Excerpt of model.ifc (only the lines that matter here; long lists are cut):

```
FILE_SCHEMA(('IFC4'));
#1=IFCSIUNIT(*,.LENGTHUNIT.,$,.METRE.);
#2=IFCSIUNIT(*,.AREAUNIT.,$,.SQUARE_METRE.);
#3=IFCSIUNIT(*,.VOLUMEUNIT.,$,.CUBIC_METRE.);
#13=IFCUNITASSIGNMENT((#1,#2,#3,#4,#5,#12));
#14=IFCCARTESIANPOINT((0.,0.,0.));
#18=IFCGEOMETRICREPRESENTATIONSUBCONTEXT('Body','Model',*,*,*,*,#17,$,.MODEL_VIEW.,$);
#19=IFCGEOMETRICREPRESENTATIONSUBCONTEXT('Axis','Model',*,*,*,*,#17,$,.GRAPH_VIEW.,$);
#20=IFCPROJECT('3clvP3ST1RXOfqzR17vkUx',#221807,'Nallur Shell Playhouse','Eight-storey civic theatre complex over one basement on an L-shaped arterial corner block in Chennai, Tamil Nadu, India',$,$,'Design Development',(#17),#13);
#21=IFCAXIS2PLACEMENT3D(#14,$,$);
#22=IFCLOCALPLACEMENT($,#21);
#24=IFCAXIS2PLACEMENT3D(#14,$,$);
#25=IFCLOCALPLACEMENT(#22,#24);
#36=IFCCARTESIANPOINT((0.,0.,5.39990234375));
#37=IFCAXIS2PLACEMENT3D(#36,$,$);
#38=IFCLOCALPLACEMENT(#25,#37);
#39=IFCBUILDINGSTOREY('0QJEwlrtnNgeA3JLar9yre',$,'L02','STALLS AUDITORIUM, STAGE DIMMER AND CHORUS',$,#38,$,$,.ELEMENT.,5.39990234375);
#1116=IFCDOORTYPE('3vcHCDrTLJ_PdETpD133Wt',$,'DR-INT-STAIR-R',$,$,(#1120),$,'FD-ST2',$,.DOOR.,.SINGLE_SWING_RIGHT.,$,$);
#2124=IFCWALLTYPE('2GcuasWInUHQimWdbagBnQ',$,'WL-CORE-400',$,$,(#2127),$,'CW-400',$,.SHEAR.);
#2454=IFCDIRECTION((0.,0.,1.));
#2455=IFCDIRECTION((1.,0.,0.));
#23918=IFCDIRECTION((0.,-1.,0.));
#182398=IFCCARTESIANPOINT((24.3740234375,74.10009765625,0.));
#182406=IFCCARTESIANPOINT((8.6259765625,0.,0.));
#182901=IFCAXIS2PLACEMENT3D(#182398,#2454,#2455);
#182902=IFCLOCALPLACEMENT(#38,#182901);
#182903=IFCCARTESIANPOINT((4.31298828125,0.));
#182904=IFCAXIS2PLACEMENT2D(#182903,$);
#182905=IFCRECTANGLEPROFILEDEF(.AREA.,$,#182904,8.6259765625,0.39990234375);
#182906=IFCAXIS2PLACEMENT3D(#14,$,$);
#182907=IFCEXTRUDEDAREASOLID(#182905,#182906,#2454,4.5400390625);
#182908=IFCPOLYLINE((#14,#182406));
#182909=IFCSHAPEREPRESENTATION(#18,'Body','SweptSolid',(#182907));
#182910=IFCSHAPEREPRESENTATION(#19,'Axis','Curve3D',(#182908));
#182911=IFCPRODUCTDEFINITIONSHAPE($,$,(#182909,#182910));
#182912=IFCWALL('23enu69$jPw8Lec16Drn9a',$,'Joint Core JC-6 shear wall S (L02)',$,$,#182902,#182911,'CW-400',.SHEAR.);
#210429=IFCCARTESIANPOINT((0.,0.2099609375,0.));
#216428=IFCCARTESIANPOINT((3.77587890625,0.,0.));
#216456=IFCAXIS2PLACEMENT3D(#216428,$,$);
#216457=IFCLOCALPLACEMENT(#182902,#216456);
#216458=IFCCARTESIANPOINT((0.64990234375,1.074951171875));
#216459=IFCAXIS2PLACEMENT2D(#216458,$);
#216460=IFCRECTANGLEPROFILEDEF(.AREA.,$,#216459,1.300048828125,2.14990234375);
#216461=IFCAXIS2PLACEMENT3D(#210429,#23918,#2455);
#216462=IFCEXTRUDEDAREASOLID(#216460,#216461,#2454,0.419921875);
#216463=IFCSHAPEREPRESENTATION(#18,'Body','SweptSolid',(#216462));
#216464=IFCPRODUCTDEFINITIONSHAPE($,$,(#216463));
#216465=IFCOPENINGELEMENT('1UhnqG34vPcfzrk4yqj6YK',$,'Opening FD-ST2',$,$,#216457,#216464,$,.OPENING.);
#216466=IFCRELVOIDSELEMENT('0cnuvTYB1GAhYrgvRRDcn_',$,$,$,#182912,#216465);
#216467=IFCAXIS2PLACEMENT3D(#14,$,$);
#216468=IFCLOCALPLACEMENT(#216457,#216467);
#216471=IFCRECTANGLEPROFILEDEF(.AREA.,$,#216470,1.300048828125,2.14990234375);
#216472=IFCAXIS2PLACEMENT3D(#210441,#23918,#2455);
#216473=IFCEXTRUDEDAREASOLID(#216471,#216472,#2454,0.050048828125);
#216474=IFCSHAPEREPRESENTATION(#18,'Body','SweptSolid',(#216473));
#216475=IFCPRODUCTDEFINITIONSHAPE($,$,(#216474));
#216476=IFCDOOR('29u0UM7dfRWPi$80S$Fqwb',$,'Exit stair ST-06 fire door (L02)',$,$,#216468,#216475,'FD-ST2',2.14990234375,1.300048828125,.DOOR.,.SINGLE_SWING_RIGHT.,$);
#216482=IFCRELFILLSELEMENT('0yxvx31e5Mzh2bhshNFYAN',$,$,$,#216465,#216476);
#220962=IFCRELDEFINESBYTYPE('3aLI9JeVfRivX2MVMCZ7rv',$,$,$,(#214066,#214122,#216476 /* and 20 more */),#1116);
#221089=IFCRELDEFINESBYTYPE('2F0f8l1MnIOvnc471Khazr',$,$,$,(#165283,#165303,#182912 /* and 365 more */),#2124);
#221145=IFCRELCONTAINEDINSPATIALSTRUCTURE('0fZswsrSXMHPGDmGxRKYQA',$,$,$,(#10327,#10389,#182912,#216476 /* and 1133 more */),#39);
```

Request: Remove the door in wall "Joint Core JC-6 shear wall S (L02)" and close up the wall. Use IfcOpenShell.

```python
import ifcopenshell
import ifcopenshell.api.feature
import ifcopenshell.api.root
import ifcopenshell.geom
import ifcopenshell.util.shape

model = ifcopenshell.open("model.ifc")
settings = ifcopenshell.geom.settings()


def volume(element):
    """Net volume in cubic metres, openings subtracted."""
    shape = ifcopenshell.geom.create_shape(settings, element)
    return ifcopenshell.util.shape.get_volume(shape.geometry)


door = model.by_guid("29u0UM7dfRWPi$80S$Fqwb")
opening = door.FillsVoids[0].RelatingOpeningElement
wall = opening.VoidsElements[0].RelatingBuildingElement
before = volume(wall)

ifcopenshell.api.root.remove_product(model, product=door)
ifcopenshell.api.feature.remove_feature(model, feature=opening)

after = volume(wall)

print(f"wall volume {before:.3f} -> {after:.3f} m3")

model.write("model_edited.ifc")
```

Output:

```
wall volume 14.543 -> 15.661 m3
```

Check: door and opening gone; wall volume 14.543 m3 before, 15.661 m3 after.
